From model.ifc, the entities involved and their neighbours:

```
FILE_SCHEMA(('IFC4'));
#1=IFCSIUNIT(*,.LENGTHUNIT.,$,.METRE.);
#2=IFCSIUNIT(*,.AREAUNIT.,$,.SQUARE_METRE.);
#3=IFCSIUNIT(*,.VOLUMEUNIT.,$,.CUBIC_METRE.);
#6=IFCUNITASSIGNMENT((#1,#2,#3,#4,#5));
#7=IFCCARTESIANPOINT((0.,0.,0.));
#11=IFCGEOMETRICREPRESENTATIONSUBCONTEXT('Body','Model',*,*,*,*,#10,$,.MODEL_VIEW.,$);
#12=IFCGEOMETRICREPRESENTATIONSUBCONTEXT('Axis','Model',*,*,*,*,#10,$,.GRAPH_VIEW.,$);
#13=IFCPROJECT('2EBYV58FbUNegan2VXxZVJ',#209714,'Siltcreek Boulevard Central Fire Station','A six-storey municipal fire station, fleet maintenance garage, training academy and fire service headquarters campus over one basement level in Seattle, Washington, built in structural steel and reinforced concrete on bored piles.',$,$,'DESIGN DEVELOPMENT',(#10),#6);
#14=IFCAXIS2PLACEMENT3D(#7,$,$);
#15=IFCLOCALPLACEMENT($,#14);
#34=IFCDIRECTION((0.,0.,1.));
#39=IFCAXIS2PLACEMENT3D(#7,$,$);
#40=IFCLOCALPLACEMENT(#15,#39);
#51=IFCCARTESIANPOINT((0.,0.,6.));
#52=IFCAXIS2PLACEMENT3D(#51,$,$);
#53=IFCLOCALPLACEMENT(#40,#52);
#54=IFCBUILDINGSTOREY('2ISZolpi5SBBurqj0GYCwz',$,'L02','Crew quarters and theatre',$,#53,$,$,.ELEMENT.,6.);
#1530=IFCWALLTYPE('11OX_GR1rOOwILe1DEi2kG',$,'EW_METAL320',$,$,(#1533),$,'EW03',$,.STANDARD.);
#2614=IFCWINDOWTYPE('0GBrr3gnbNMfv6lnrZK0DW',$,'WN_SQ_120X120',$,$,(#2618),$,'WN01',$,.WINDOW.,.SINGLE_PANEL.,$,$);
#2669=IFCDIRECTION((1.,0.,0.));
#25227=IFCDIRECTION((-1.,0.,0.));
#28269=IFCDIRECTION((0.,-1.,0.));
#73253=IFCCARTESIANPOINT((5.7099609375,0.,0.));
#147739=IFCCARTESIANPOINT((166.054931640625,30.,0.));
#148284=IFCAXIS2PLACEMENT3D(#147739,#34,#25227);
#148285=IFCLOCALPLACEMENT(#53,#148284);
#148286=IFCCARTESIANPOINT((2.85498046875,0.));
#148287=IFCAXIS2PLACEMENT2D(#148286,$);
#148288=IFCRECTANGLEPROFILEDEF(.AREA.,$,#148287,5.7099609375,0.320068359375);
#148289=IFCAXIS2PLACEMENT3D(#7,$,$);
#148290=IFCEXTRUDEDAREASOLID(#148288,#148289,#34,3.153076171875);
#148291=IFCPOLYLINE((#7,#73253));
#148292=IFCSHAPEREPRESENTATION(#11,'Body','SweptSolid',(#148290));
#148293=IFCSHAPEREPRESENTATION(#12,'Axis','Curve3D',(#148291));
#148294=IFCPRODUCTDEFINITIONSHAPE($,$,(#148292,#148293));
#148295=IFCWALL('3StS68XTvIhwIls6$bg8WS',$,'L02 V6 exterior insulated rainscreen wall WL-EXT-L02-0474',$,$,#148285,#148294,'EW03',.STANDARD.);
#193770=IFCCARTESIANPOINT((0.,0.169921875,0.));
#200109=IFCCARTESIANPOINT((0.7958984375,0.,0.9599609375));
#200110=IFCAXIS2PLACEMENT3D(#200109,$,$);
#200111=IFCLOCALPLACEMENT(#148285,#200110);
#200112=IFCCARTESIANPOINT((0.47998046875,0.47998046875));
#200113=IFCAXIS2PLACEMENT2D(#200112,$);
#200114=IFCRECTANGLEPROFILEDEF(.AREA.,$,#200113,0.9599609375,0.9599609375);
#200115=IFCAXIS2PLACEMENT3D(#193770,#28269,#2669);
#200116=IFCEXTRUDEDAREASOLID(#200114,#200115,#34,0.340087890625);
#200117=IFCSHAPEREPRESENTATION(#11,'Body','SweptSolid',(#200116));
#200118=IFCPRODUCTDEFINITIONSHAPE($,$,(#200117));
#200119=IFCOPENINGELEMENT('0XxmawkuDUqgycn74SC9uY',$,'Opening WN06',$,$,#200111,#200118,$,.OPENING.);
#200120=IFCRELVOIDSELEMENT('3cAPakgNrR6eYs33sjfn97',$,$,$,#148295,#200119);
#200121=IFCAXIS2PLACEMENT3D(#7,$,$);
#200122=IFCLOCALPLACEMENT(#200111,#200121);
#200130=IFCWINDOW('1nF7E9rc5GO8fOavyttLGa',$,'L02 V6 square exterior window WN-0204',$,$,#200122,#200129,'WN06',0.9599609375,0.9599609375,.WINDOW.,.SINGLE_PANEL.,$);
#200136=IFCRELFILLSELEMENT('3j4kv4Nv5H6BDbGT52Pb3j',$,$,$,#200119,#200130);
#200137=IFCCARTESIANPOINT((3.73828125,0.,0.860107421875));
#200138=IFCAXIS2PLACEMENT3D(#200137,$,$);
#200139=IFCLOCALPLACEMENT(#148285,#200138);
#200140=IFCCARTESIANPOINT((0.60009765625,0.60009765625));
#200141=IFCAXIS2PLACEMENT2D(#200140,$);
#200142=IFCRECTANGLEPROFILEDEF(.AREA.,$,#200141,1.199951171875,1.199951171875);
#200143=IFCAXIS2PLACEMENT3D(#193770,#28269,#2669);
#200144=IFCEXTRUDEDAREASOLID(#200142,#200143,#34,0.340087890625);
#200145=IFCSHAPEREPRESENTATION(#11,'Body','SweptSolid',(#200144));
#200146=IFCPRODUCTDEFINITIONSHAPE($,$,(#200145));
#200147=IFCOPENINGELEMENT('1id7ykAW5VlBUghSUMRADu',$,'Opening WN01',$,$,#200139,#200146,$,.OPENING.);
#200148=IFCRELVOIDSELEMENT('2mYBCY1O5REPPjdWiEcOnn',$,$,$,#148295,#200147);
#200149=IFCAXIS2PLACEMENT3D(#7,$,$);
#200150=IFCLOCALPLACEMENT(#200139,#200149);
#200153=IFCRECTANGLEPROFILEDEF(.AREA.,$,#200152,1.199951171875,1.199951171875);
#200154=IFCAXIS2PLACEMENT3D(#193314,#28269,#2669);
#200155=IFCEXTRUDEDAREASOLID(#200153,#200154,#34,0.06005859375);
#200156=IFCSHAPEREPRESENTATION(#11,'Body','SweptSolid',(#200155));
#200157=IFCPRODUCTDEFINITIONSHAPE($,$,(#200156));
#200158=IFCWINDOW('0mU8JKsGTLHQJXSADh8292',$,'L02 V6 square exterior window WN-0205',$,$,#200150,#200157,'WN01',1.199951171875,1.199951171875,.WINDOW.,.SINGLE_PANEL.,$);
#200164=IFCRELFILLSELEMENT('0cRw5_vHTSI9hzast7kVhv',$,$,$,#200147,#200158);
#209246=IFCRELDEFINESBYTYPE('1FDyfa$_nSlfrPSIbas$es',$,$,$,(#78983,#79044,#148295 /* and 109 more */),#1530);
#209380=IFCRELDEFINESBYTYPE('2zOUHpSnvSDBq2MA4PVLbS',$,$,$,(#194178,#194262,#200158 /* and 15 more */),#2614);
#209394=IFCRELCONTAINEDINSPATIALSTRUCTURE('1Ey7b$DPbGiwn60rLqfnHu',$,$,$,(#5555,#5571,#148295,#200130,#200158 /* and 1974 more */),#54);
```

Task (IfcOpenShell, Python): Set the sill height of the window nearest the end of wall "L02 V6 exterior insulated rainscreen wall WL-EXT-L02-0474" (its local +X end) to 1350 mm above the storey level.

```python
import numpy as np
import ifcopenshell
import ifcopenshell.api.geometry
import ifcopenshell.geom
import ifcopenshell.util.element
import ifcopenshell.util.placement
import ifcopenshell.util.shape
import ifcopenshell.util.unit

model = ifcopenshell.open("model.ifc")
unit_scale = ifcopenshell.util.unit.calculate_unit_scale(model)

window = model.by_guid("0mU8JKsGTLHQJXSADh8292")
opening = window.FillsVoids[0].RelatingOpeningElement
storey = ifcopenshell.util.element.get_container(window, ifc_class="IfcBuildingStorey")
level = ifcopenshell.util.placement.get_local_placement(storey.ObjectPlacement)[2, 3]

# The opening's origin need not be at the sill, so measure its lowest point.
shape = ifcopenshell.geom.create_shape(ifcopenshell.geom.settings(), opening)
bottom = ifcopenshell.util.shape.get_shape_bottom_elevation(shape, shape.geometry) / unit_scale
dz = level + 1.35 / unit_scale - bottom

shift = np.array([0.0, 0.0, dz])
# The window is placed relative to its opening, so it follows when the opening moves.
matrix = ifcopenshell.util.placement.get_local_placement(opening.ObjectPlacement)
matrix[:3, 3] += shift
ifcopenshell.api.geometry.edit_object_placement(
    model, product=opening, matrix=matrix, is_si=False, should_transform_children=True
)

print(f"moved by {dz * unit_scale:+.3f} m")

model.write("model_updated.ifc")
```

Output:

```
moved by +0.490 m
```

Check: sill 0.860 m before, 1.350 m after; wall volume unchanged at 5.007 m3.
